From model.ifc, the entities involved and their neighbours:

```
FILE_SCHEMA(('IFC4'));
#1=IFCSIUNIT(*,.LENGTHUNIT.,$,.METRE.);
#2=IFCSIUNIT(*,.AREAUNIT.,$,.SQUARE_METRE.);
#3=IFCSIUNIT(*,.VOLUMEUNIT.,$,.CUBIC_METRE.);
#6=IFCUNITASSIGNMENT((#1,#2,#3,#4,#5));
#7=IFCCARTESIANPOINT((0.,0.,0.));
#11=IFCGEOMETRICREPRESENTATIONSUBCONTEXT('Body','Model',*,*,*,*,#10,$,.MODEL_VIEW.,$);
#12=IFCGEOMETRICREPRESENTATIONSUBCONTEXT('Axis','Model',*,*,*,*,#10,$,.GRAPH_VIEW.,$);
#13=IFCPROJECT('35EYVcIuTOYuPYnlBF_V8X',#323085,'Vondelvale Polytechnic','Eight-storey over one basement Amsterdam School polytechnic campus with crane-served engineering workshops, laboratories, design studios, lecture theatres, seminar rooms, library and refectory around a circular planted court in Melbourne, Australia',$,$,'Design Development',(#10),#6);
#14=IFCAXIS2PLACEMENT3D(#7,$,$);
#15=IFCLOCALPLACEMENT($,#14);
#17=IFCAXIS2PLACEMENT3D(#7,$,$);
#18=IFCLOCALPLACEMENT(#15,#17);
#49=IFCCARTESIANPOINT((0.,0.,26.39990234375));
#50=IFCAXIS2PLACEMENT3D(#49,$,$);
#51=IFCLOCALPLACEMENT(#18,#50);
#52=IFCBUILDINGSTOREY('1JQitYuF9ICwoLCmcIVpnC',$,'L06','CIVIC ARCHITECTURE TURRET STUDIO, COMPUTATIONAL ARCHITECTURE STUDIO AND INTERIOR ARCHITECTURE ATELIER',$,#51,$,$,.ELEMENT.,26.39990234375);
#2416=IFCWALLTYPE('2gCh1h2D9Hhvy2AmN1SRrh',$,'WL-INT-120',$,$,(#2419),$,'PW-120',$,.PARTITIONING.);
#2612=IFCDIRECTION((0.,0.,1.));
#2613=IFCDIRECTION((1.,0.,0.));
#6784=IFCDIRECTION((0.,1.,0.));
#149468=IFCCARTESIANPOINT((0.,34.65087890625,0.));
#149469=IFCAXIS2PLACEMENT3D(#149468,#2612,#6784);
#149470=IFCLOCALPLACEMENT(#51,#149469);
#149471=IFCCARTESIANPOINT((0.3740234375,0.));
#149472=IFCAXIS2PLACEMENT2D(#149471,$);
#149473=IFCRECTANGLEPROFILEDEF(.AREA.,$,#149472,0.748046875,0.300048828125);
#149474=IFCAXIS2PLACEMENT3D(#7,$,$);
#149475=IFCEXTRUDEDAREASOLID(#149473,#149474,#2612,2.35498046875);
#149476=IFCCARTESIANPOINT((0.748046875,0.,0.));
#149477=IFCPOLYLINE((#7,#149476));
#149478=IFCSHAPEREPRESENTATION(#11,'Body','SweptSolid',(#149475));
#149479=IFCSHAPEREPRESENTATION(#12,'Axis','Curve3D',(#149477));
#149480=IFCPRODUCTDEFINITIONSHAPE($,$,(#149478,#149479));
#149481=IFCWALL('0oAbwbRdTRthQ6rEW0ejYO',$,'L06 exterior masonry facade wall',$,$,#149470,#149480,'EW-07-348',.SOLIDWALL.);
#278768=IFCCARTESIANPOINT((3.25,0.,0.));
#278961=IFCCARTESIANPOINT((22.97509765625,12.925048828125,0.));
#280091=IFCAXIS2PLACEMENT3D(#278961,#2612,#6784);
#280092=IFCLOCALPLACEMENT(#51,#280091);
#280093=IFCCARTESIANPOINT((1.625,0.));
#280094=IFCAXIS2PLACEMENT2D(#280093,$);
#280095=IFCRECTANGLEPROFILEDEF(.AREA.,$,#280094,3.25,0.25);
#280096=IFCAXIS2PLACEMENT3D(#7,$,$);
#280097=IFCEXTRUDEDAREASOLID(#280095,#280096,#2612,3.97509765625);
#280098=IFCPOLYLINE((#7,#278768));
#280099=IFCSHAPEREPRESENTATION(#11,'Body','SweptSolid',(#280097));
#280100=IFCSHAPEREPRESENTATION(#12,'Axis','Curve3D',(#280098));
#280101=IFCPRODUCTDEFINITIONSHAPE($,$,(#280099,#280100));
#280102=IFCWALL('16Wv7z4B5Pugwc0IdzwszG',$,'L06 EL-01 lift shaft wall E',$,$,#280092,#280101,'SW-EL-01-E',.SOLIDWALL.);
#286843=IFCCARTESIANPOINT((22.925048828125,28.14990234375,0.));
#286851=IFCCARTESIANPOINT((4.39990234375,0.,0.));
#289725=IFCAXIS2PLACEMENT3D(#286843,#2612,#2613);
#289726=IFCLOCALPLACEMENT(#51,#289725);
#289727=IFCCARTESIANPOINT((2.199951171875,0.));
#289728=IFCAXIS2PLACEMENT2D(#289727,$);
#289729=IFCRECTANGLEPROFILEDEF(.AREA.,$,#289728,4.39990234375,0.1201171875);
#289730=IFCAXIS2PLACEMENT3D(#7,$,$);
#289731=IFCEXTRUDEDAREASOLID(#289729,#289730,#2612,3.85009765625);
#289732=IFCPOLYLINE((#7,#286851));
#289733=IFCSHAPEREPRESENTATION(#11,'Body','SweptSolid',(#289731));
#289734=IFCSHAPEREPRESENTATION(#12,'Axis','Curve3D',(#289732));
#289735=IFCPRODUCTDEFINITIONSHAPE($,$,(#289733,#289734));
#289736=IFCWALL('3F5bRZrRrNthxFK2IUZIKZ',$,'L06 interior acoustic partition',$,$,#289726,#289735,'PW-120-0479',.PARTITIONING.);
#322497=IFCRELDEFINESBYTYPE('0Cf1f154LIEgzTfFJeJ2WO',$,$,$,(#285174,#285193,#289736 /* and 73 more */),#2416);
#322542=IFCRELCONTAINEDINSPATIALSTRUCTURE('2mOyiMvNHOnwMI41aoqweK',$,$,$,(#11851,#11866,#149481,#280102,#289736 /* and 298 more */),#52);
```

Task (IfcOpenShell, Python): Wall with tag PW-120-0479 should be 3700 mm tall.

```python
import ifcopenshell
import ifcopenshell.geom
import ifcopenshell.util.representation
import ifcopenshell.util.shape
import ifcopenshell.util.unit

model = ifcopenshell.open("model.ifc")
unit_scale = ifcopenshell.util.unit.calculate_unit_scale(model)
settings = ifcopenshell.geom.settings()


def volume(element):
    """Net volume in cubic metres, openings subtracted."""
    shape = ifcopenshell.geom.create_shape(settings, element)
    return ifcopenshell.util.shape.get_volume(shape.geometry)


wall = model.by_guid("3F5bRZrRrNthxFK2IUZIKZ")
before = volume(wall)

body = ifcopenshell.util.representation.get_representation(wall, "Model", "Body")
solid = body.Items[0]
old_height = solid.Depth
solid.Depth = 3.7 / unit_scale
after = volume(wall)

print(f"height {old_height:g} -> {solid.Depth:g}, volume {before:.3f} -> {after:.3f} m3")

model.write("model_updated.ifc")
```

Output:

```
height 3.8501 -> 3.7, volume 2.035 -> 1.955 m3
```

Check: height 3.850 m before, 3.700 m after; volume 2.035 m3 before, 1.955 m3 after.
